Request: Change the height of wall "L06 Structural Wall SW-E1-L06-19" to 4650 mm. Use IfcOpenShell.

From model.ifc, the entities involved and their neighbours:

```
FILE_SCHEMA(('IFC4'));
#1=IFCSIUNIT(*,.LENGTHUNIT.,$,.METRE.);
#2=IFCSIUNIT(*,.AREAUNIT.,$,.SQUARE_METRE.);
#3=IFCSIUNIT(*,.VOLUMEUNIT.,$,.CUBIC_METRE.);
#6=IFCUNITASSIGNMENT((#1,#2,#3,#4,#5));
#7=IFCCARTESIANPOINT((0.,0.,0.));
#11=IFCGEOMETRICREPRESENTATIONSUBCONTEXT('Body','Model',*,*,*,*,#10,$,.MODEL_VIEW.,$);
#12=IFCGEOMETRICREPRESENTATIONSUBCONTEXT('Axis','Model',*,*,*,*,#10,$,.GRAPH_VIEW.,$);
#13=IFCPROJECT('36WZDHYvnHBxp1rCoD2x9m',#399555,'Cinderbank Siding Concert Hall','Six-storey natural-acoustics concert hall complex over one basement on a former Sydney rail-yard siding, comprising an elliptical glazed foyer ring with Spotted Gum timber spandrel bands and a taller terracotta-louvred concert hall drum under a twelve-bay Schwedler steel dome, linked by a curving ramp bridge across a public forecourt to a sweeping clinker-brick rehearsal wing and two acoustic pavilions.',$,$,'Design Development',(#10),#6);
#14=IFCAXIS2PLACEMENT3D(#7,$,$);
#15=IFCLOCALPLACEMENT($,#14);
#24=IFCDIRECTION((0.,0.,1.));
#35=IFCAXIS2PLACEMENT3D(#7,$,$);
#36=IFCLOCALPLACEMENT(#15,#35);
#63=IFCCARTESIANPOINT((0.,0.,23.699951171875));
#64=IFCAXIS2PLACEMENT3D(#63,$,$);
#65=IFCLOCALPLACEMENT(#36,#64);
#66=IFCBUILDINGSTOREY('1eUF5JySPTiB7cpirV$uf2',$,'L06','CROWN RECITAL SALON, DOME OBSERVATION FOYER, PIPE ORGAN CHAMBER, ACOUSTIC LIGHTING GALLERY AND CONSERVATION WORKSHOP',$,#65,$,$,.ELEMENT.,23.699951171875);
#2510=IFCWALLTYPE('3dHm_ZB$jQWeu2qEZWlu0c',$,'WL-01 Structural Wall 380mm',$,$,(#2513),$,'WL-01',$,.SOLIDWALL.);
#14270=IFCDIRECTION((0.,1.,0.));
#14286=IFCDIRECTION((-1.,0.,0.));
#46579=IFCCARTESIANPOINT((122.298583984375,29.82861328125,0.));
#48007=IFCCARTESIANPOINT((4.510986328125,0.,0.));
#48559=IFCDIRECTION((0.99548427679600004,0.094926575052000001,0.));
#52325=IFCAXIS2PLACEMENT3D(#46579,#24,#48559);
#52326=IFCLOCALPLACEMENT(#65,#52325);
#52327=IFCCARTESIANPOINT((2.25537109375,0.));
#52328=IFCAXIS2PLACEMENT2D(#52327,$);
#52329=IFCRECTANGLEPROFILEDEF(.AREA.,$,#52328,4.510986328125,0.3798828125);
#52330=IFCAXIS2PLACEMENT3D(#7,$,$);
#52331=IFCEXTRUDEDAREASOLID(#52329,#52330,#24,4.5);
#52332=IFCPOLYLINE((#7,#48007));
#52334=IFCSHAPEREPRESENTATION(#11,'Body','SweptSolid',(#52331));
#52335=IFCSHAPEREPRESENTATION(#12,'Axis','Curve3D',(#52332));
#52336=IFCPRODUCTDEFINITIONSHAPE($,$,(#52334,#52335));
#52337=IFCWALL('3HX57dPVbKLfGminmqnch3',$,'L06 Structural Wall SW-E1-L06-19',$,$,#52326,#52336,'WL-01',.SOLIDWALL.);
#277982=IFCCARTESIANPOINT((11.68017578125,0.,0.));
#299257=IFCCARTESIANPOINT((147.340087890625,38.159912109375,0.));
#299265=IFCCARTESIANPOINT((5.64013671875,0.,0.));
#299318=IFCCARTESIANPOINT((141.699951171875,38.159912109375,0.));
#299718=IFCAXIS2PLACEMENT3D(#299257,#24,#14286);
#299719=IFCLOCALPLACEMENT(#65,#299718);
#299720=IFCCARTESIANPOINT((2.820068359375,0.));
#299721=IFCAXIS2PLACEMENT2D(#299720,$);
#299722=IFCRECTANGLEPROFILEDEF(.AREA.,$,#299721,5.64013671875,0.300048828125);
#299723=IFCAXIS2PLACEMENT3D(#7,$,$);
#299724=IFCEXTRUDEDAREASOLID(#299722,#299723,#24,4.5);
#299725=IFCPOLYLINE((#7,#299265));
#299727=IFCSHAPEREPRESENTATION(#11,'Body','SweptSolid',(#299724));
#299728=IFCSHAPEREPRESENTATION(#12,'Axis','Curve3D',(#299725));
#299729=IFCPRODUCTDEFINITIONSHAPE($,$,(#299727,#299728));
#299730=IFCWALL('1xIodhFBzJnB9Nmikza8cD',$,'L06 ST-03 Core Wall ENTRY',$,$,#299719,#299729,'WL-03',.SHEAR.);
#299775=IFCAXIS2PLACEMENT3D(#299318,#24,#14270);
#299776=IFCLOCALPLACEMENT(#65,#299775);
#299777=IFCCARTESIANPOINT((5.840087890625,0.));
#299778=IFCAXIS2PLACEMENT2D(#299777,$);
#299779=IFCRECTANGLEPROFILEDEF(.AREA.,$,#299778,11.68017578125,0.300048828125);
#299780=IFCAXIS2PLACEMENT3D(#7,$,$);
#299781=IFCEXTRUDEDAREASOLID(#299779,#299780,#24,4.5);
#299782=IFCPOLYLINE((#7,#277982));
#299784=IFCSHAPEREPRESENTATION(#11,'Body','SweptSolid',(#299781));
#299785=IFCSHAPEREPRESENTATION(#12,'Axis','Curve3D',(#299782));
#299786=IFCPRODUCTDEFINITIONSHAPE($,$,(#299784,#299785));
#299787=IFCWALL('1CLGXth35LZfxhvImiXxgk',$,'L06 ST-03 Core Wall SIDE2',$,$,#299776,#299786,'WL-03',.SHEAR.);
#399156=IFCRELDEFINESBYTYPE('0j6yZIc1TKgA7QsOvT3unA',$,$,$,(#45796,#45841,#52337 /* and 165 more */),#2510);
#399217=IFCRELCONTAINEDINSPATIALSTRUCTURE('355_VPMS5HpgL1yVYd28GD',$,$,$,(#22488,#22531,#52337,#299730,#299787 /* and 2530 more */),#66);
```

```python
import ifcopenshell
import ifcopenshell.geom
import ifcopenshell.util.representation
import ifcopenshell.util.shape

model = ifcopenshell.open("model.ifc")
settings = ifcopenshell.geom.settings()


def volume(element):
    """Net volume in cubic metres, openings subtracted."""
    shape = ifcopenshell.geom.create_shape(settings, element)
    return ifcopenshell.util.shape.get_volume(shape.geometry)


wall = model.by_id(52337)
before = volume(wall)

body = ifcopenshell.util.representation.get_representation(wall, "Model", "Body")
solid = body.Items[0]
old_height = solid.Depth
solid.Depth = 4.65
after = volume(wall)

print(f"height {old_height:g} -> {solid.Depth:g}, volume {before:.3f} -> {after:.3f} m3")

model.write("model_edited.ifc")
```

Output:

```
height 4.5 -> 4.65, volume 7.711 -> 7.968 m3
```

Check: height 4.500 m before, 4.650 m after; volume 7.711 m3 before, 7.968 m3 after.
